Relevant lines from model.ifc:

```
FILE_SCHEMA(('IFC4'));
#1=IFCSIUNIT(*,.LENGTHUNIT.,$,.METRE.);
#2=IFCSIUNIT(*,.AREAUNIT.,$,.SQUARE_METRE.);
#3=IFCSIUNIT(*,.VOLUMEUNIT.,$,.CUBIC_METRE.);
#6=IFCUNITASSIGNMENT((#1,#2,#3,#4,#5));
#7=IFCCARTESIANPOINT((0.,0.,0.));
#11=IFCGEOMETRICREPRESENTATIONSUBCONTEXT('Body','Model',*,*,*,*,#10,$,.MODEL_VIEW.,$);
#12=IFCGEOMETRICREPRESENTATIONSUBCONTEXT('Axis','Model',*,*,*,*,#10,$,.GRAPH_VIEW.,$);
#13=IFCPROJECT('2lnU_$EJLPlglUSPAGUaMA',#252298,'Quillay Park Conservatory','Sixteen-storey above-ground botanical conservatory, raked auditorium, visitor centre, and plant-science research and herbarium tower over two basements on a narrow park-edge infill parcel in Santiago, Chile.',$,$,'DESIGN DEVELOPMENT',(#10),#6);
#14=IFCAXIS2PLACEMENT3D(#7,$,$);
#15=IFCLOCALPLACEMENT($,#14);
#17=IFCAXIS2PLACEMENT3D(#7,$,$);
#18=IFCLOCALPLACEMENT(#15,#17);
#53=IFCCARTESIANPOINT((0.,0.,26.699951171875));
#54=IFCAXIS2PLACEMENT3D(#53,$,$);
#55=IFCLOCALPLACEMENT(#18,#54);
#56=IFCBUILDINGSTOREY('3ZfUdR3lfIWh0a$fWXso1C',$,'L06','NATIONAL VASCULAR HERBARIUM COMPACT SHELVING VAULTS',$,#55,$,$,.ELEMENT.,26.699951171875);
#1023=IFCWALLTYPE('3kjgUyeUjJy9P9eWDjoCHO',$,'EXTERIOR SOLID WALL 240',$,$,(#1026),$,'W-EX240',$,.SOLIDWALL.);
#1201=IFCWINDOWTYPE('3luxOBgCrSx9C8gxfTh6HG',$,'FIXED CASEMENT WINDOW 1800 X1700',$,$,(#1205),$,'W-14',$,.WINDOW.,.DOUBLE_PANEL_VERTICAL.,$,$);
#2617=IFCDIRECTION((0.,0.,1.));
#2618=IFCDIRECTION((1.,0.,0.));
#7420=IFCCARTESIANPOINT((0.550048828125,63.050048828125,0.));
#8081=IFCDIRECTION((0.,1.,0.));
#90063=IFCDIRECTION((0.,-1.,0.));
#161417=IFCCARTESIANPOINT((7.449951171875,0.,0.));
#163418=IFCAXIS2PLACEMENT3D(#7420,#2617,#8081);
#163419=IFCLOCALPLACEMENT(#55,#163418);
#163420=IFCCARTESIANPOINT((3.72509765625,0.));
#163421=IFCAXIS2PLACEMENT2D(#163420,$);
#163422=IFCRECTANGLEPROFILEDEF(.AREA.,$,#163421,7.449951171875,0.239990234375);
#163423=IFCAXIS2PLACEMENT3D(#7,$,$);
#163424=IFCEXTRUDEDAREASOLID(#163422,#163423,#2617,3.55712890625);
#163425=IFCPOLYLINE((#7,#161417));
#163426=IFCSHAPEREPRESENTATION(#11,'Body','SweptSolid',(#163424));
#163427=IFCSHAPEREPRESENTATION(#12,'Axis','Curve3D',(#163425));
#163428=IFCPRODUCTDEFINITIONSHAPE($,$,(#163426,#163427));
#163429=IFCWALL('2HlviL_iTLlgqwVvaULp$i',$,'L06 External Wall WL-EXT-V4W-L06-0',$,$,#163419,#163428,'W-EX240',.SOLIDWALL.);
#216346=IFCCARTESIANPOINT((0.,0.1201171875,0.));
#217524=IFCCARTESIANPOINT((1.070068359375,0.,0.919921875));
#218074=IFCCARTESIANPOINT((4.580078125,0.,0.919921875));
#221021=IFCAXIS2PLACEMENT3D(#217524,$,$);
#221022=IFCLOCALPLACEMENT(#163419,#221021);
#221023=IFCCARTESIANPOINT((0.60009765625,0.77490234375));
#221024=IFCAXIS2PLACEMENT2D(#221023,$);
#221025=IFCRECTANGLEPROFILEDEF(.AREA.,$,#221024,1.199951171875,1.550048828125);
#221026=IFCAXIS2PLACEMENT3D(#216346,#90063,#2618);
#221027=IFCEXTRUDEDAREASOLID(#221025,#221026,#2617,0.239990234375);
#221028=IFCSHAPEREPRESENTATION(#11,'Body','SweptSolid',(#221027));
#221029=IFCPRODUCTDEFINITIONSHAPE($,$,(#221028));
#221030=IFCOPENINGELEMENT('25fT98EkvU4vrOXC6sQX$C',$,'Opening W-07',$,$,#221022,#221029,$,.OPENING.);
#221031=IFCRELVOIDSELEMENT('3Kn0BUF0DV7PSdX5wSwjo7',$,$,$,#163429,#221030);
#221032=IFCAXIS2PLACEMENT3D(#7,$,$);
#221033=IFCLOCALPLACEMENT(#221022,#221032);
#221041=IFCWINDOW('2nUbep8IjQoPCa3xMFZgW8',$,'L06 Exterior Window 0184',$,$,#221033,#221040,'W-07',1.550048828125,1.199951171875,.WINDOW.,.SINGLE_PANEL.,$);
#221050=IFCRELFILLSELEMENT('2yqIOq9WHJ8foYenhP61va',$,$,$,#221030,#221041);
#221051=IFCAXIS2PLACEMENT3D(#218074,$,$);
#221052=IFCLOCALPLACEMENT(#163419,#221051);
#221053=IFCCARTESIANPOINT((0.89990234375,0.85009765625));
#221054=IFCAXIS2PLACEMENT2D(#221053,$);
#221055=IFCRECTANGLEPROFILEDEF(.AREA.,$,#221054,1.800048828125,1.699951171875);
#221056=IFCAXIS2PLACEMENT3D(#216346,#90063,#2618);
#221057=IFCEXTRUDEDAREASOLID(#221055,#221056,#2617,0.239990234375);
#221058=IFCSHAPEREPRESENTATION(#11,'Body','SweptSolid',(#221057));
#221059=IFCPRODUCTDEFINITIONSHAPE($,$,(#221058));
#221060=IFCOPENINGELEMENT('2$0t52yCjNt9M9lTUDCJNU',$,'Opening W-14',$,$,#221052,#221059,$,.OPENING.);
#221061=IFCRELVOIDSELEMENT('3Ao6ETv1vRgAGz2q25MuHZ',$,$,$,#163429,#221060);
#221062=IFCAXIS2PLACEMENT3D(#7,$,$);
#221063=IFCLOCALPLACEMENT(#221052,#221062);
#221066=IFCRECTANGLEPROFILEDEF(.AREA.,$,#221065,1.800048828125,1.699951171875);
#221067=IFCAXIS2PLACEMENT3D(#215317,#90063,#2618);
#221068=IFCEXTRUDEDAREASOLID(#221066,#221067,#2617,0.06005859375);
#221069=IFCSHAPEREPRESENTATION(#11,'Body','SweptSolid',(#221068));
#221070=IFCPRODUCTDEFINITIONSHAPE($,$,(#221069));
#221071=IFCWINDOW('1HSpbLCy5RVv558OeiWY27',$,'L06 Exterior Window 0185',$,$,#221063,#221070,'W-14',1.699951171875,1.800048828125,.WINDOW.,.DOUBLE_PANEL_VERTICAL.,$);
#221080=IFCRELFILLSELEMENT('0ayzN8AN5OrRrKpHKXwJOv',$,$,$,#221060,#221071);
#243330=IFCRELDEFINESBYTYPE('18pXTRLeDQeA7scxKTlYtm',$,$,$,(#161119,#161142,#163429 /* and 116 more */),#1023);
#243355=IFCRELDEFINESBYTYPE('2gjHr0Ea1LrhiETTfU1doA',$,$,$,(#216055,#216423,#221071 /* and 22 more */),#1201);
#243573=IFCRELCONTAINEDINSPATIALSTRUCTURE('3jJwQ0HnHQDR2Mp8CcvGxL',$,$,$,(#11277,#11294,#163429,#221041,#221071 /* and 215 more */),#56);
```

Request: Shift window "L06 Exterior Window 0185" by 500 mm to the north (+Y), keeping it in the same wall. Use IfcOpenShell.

```python
import ifcopenshell
import ifcopenshell.api.geometry
import ifcopenshell.util.placement
import ifcopenshell.util.unit

model = ifcopenshell.open("model.ifc")
unit_scale = ifcopenshell.util.unit.calculate_unit_scale(model)

window = model.by_guid("1HSpbLCy5RVv558OeiWY27")
opening = window.FillsVoids[0].RelatingOpeningElement
wall = opening.VoidsElements[0].RelatingBuildingElement

wall_matrix = ifcopenshell.util.placement.get_local_placement(wall.ObjectPlacement)
shift = wall_matrix[:3, 0] * 0.5 / unit_scale
before = ifcopenshell.util.placement.get_local_placement(window.ObjectPlacement)[:3, 3].copy()

# The window is placed relative to its opening, so it follows when the opening moves.
matrix = ifcopenshell.util.placement.get_local_placement(opening.ObjectPlacement)
matrix[:3, 3] += shift
ifcopenshell.api.geometry.edit_object_placement(
    model, product=opening, matrix=matrix, is_si=False, should_transform_children=True
)

after = ifcopenshell.util.placement.get_local_placement(window.ObjectPlacement)[:3, 3]
print("window moved by", (after - before).round(3) + 0.0)

model.write("model_rev.ifc")
```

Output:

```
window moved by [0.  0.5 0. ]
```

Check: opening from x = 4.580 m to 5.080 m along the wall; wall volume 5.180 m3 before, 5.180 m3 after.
